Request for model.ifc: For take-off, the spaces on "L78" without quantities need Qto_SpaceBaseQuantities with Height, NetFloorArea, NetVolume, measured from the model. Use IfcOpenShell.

First a look at what the model holds.

```python
import ifcopenshell
import ifcopenshell.util.element
import ifcopenshell.util.unit

model = ifcopenshell.open("model.ifc")
print(model.schema)
for unit_type in ("LENGTHUNIT", "AREAUNIT", "VOLUMEUNIT"):
    print(unit_type, ifcopenshell.util.unit.calculate_unit_scale(model, unit_type))
storey = next(s for s in model.by_type("IfcBuildingStorey") if s.Name == "L78")
spaces = [e for e in ifcopenshell.util.element.get_decomposition(storey) if e.is_a("IfcSpace")]
for e in sorted(spaces, key=lambda e: e.id()):
    print(e.id(), e.is_a(), e.Name, list(ifcopenshell.util.element.get_psets(e, qtos_only=True)), sep=" | ")
```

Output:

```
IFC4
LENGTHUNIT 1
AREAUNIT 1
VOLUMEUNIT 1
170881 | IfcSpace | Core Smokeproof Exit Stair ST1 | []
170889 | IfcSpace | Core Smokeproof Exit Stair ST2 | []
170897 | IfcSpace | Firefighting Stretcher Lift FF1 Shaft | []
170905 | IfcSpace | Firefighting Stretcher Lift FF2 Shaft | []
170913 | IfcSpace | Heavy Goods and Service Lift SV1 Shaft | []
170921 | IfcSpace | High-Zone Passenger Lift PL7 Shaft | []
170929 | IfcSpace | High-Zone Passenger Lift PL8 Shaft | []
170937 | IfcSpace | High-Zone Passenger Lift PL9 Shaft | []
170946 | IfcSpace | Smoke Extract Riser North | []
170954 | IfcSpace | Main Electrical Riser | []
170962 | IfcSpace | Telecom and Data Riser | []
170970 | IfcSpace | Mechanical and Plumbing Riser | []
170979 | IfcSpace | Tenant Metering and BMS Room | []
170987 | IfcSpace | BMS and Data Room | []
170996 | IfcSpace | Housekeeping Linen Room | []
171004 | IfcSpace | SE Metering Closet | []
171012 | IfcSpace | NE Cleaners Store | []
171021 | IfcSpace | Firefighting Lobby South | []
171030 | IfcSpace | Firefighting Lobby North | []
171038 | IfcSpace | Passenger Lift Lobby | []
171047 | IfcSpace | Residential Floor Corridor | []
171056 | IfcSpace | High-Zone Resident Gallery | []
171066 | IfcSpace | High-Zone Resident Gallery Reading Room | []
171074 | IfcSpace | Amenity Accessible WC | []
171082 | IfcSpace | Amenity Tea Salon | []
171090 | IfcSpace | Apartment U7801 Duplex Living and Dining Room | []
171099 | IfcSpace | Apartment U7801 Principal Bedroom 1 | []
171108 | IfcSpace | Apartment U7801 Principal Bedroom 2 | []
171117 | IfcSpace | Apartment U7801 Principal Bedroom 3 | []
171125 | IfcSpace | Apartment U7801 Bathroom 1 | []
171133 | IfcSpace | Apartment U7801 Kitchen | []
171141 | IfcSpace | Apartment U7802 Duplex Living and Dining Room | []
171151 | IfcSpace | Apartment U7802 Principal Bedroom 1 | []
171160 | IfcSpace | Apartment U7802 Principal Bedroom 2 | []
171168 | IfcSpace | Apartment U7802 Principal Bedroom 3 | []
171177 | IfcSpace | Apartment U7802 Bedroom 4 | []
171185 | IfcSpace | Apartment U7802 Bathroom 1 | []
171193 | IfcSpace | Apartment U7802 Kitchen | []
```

```python
import ifcopenshell
import ifcopenshell.api.pset
import ifcopenshell.geom
import ifcopenshell.util.element
import ifcopenshell.util.shape
import ifcopenshell.util.unit

model = ifcopenshell.open("model.ifc")
unit_scale = ifcopenshell.util.unit.calculate_unit_scale(model)
area_scale = ifcopenshell.util.unit.calculate_unit_scale(model, "AREAUNIT")
volume_scale = ifcopenshell.util.unit.calculate_unit_scale(model, "VOLUMEUNIT")
settings = ifcopenshell.geom.settings()

storey = next(s for s in model.by_type("IfcBuildingStorey") if s.Name == "L78")
spaces = [e for e in ifcopenshell.util.element.get_decomposition(storey) if e.is_a("IfcSpace")]

for e in sorted(spaces, key=lambda e: e.id()):
    if ifcopenshell.util.element.get_psets(e, qtos_only=True, should_inherit=False):
        continue
    # Geometry comes back in metres, in the element's own axes.
    shape = ifcopenshell.geom.create_shape(settings, e)
    values = {
        "Height": ifcopenshell.util.shape.get_z(shape.geometry) / unit_scale,
        "NetFloorArea": ifcopenshell.util.shape.get_footprint_area(shape.geometry) / area_scale,
        "NetVolume": ifcopenshell.util.shape.get_volume(shape.geometry) / volume_scale,
    }
    qto = ifcopenshell.api.pset.add_qto(model, product=e, name="Qto_SpaceBaseQuantities")
    ifcopenshell.api.pset.edit_qto(model, qto=qto, properties=values)
    print(e.id(), {k: round(v, 3) for k, v in values.items()})

model.write("model-out.ifc")
```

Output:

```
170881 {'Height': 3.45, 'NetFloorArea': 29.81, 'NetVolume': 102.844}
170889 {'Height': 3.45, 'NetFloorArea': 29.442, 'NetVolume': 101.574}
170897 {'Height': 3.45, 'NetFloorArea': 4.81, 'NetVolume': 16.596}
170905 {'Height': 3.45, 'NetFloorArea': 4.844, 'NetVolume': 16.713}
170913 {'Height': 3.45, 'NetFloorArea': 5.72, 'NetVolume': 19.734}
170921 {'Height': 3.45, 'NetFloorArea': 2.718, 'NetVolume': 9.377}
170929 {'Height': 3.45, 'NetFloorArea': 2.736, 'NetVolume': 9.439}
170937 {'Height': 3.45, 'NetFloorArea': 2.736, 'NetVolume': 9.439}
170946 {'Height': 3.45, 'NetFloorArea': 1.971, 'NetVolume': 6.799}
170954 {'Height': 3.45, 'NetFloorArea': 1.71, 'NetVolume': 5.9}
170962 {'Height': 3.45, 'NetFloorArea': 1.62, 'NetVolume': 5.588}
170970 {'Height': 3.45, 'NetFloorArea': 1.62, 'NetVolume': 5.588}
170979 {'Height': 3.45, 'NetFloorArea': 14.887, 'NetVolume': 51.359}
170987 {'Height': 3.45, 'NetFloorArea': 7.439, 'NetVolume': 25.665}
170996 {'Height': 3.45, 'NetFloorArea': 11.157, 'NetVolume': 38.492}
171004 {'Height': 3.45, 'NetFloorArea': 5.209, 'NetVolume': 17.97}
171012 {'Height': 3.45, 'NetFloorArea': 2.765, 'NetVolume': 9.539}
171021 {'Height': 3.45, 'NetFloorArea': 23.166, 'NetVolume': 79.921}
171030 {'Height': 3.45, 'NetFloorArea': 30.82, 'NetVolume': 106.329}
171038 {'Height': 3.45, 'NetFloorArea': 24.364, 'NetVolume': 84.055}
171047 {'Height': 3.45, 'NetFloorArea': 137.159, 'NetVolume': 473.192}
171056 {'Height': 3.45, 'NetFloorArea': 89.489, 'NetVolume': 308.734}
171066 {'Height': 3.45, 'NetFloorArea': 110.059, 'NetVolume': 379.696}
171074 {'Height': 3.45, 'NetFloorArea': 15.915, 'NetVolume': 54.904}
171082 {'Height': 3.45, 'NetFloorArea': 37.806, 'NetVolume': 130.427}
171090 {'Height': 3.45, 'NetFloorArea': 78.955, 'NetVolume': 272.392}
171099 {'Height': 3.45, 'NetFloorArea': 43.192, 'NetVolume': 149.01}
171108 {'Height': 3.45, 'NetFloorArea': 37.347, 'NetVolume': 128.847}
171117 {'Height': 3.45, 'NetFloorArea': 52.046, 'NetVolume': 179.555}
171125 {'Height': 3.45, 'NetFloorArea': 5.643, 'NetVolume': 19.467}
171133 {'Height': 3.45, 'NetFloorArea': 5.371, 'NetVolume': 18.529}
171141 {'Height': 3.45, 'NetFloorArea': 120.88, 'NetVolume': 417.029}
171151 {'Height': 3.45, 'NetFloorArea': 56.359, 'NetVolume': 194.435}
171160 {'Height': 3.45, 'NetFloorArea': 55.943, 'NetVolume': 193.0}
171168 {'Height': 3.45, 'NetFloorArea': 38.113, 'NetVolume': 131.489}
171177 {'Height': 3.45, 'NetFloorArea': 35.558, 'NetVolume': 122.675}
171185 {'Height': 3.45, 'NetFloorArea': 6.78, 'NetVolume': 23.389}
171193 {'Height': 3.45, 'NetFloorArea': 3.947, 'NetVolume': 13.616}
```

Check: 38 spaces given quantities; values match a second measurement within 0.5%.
